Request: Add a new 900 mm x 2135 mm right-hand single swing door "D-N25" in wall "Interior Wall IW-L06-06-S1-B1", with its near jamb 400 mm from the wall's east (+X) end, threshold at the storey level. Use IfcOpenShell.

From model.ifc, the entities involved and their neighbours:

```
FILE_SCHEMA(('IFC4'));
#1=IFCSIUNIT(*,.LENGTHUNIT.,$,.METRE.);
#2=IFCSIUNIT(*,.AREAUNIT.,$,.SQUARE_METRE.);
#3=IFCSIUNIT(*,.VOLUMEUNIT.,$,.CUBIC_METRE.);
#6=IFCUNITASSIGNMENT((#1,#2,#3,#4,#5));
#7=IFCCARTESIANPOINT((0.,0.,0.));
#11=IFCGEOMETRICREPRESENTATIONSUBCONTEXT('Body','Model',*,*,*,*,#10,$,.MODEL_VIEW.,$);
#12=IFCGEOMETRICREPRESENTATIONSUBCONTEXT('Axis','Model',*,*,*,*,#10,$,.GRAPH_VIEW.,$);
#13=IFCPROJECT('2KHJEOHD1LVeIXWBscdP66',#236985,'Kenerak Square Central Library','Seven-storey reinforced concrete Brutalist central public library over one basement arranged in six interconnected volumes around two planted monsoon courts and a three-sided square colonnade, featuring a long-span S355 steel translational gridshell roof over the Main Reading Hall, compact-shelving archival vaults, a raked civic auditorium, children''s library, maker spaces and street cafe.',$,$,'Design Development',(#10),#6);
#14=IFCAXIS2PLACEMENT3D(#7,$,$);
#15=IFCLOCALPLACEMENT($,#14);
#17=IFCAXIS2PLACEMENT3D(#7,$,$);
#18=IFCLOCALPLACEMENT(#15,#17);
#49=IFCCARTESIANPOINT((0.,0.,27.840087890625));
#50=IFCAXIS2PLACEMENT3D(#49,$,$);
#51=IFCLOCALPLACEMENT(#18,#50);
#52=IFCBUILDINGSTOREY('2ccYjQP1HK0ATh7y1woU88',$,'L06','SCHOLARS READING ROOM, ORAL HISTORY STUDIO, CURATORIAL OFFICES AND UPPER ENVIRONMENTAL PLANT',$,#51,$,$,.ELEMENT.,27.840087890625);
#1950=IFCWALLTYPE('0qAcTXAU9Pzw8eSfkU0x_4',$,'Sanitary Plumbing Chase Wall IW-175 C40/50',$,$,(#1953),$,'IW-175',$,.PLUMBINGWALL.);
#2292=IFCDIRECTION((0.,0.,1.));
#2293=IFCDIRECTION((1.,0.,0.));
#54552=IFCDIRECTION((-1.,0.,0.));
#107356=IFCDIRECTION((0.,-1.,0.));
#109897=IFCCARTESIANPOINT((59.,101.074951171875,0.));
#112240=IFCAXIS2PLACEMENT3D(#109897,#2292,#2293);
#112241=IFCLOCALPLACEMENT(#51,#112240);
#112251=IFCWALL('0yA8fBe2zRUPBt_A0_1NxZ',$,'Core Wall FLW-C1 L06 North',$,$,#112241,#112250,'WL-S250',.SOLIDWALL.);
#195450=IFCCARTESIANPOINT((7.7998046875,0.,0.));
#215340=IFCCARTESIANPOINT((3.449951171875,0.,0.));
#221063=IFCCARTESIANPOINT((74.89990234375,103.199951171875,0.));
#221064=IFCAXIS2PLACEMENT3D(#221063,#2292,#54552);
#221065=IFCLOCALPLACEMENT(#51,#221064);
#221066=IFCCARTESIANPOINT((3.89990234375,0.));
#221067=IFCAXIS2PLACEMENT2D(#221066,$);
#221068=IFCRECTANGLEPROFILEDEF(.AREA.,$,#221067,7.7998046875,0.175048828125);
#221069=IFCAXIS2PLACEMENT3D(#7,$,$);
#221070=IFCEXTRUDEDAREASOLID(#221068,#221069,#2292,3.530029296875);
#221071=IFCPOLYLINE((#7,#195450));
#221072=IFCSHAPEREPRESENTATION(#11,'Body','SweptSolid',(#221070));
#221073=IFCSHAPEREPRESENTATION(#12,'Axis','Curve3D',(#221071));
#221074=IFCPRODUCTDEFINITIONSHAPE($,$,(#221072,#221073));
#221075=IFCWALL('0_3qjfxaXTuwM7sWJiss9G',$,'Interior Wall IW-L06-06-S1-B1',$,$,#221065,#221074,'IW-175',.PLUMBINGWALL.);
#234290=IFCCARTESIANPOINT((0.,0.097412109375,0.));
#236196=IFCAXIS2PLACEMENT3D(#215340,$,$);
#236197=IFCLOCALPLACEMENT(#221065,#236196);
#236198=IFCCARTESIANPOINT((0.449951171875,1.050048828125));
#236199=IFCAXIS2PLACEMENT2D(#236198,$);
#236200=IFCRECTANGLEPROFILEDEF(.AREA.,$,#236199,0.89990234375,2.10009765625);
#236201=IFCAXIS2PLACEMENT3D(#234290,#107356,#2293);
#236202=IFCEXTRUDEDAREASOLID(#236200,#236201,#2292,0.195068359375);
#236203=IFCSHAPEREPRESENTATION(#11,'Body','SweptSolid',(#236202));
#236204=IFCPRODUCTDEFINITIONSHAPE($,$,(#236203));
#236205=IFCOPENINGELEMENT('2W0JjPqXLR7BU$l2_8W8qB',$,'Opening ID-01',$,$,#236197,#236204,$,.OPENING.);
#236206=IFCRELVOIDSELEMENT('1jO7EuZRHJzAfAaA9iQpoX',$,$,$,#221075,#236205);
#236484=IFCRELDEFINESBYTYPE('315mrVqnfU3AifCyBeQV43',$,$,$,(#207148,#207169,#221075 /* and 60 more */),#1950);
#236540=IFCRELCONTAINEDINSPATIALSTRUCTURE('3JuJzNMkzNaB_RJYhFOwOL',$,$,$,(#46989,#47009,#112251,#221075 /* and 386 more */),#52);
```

```python
import numpy as np
import ifcopenshell
import ifcopenshell.api.feature
import ifcopenshell.api.geometry
import ifcopenshell.api.root
import ifcopenshell.api.spatial
import ifcopenshell.geom
import ifcopenshell.util.element
import ifcopenshell.util.placement
import ifcopenshell.util.representation
import ifcopenshell.util.shape
import ifcopenshell.util.unit

model = ifcopenshell.open("model.ifc")
unit_scale = ifcopenshell.util.unit.calculate_unit_scale(model)
settings = ifcopenshell.geom.settings()


def volume(element):
    """Net volume in cubic metres, openings subtracted."""
    shape = ifcopenshell.geom.create_shape(settings, element)
    return ifcopenshell.util.shape.get_volume(shape.geometry)


wall = model.by_guid("0_3qjfxaXTuwM7sWJiss9G")
storey = ifcopenshell.util.element.get_container(wall, ifc_class="IfcBuildingStorey")
context = ifcopenshell.util.representation.get_context(model, "Model", "Body", "MODEL_VIEW")
before = volume(wall)

width, height, from_end, sill = 0.9, 2.135, 0.4, 0.0  # metres

# The wall runs along its own X axis, and the end named is its -X end.
wall_shape = ifcopenshell.geom.create_shape(settings, wall)
x, y, z = ifcopenshell.util.shape.get_vertices(wall_shape.geometry).T
start = x.min() + from_end
face, thickness = float(y.min()), float(y.max() - y.min())
wall_matrix = ifcopenshell.util.placement.get_local_placement(wall.ObjectPlacement)
level = ifcopenshell.util.placement.get_local_placement(storey.ObjectPlacement)[2, 3]


def in_wall(x, y):
    """Placement at x, y metres in the wall's axes, at sill height."""
    matrix = wall_matrix.copy()
    matrix[:, 3] = wall_matrix @ np.array([x / unit_scale, y / unit_scale, 0.0, 1.0])
    matrix[2, 3] = level + sill / unit_scale
    return matrix


# Opening: a box that overshoots both wall faces by 50 mm.
opening = ifcopenshell.api.root.create_entity(model, ifc_class="IfcOpeningElement", predefined_type="OPENING")
box = ifcopenshell.api.geometry.add_wall_representation(
    model, context=context, length=width, height=height, thickness=thickness + 0.1
)
ifcopenshell.api.geometry.assign_representation(model, product=opening, representation=box)
ifcopenshell.api.geometry.edit_object_placement(model, product=opening, matrix=in_wall(start, face - 0.05), is_si=False)
ifcopenshell.api.feature.add_feature(model, feature=opening, element=wall)

door = ifcopenshell.api.root.create_entity(model, ifc_class="IfcDoor", name="D-N25", predefined_type="DOOR")
door.OverallWidth, door.OverallHeight = width / unit_scale, height / unit_scale
door.OperationType = "SINGLE_SWING_RIGHT"
body = ifcopenshell.api.geometry.add_door_representation(
    model,
    context=context,
    overall_width=door.OverallWidth,
    overall_height=door.OverallHeight,
    operation_type="SINGLE_SWING_RIGHT",
    lining_properties={"LiningDepth": thickness / unit_scale, "ThresholdDepth": thickness / unit_scale},
)
ifcopenshell.api.geometry.assign_representation(model, product=door, representation=body)
ifcopenshell.api.spatial.assign_container(model, products=[door], relating_structure=storey)
ifcopenshell.api.feature.add_filling(model, opening=opening, element=door)

# The lining spans the wall, so the door starts at the wall face.
ifcopenshell.api.geometry.edit_object_placement(model, product=door, matrix=in_wall(start, face), is_si=False)

after = volume(wall)

print(f"wall volume {before:.3f} -> {after:.3f} m3")

model.write("model-out.ifc")
```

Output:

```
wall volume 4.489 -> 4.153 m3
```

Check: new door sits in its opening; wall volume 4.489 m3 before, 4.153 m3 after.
